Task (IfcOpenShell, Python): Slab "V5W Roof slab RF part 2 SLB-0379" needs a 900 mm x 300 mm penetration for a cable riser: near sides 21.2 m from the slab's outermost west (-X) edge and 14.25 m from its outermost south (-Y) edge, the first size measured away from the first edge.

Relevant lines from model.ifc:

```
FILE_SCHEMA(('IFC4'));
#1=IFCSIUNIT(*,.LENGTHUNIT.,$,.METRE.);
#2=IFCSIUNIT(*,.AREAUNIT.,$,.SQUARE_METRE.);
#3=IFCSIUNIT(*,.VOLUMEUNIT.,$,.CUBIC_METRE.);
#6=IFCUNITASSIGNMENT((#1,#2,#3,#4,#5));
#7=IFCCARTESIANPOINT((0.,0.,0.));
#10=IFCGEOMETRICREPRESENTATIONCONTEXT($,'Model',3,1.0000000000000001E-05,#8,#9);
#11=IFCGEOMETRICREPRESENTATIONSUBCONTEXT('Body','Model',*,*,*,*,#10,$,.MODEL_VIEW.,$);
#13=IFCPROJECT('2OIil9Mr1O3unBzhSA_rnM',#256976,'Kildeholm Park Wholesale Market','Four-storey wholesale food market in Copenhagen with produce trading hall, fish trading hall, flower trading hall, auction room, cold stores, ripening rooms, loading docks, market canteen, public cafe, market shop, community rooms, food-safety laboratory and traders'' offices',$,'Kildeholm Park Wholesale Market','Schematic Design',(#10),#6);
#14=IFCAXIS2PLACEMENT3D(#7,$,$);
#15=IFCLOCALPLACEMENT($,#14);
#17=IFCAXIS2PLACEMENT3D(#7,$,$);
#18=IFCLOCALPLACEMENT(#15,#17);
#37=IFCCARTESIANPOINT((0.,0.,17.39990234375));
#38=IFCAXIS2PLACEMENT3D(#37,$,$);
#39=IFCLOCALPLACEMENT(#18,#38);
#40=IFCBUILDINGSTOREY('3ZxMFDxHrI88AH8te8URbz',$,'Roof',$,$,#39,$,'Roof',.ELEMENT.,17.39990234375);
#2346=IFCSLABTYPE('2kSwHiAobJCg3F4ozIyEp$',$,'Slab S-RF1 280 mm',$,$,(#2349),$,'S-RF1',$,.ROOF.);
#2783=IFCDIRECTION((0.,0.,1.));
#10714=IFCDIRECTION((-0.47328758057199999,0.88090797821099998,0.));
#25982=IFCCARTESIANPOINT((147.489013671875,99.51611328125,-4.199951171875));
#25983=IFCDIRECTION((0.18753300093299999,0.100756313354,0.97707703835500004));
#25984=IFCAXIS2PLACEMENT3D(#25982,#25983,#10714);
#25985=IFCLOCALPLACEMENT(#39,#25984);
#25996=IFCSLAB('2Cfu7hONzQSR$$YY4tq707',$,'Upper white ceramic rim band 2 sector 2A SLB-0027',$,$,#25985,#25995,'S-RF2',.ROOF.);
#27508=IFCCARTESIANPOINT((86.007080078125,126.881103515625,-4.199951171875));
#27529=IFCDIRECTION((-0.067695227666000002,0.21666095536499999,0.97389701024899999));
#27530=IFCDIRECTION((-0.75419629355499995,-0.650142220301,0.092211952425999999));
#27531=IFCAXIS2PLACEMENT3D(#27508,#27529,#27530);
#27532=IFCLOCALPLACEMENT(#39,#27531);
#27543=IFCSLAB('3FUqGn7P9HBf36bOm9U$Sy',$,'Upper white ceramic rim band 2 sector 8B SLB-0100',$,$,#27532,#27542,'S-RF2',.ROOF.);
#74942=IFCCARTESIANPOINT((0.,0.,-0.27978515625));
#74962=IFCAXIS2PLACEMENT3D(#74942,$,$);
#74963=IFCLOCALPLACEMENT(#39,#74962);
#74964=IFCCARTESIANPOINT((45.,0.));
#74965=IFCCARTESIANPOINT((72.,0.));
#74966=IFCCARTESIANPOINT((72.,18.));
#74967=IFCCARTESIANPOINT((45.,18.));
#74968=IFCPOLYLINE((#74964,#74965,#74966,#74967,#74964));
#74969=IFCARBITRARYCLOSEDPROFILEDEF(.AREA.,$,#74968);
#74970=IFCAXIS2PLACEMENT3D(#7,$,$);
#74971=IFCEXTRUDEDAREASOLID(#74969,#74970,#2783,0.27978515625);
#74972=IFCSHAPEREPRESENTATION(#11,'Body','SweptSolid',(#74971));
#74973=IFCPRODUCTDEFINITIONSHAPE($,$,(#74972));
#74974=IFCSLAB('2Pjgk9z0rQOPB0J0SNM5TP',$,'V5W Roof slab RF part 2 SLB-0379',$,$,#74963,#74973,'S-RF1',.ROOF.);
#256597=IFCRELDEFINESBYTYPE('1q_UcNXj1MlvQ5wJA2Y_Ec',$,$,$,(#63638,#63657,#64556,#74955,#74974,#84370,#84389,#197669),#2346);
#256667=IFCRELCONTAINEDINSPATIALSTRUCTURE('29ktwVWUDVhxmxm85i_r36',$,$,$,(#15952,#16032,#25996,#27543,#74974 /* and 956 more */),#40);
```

```python
import numpy as np
import ifcopenshell
import ifcopenshell.api.feature
import ifcopenshell.api.geometry
import ifcopenshell.api.root
import ifcopenshell.geom
import ifcopenshell.util.placement
import ifcopenshell.util.representation
import ifcopenshell.util.shape
import ifcopenshell.util.unit

model = ifcopenshell.open("model.ifc")
unit_scale = ifcopenshell.util.unit.calculate_unit_scale(model)
settings = ifcopenshell.geom.settings()


def volume(element):
    """Net volume in cubic metres, openings subtracted."""
    shape = ifcopenshell.geom.create_shape(settings, element)
    return ifcopenshell.util.shape.get_volume(shape.geometry)


slab = model.by_guid("2Pjgk9z0rQOPB0J0SNM5TP")
before = volume(slab)

# Extent in the slab's own axes, in metres. The edges named are its -X and -Y sides.
slab_shape = ifcopenshell.geom.create_shape(settings, slab)
vertices = ifcopenshell.util.shape.get_vertices(slab_shape.geometry)
x_min, y_min, bottom = vertices.min(axis=0)
top = vertices[:, 2].max()

opening = ifcopenshell.api.root.create_entity(model, ifc_class="IfcOpeningElement", name="Cable riser opening", predefined_type="OPENING")
context = ifcopenshell.util.representation.get_context(model, "Model", "Body", "MODEL_VIEW")
width, depth = 0.9, 0.3
outline = [(0.0, 0.0), (width, 0.0), (width, depth), (0.0, depth), (0.0, 0.0)]
# Overshoot both faces by 50 mm so the cut is clean.
shape = ifcopenshell.api.geometry.add_slab_representation(
    model, context=context, depth=top - bottom + 0.1, polyline=outline
)
ifcopenshell.api.geometry.assign_representation(model, product=opening, representation=shape)

matrix = ifcopenshell.util.placement.get_local_placement(slab.ObjectPlacement)
matrix[:, 3] = matrix @ np.append(np.array([x_min + 21.2, y_min + 14.25, bottom - 0.05]) / unit_scale, 1.0)
ifcopenshell.api.geometry.edit_object_placement(model, product=opening, matrix=matrix, is_si=False)
ifcopenshell.api.feature.add_feature(model, feature=opening, element=slab)

after = volume(slab)

print(f"slab volume {before:.3f} -> {after:.3f} m3")

model.write("model_updated.ifc")
```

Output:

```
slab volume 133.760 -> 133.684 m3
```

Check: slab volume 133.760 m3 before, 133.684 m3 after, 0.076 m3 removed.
